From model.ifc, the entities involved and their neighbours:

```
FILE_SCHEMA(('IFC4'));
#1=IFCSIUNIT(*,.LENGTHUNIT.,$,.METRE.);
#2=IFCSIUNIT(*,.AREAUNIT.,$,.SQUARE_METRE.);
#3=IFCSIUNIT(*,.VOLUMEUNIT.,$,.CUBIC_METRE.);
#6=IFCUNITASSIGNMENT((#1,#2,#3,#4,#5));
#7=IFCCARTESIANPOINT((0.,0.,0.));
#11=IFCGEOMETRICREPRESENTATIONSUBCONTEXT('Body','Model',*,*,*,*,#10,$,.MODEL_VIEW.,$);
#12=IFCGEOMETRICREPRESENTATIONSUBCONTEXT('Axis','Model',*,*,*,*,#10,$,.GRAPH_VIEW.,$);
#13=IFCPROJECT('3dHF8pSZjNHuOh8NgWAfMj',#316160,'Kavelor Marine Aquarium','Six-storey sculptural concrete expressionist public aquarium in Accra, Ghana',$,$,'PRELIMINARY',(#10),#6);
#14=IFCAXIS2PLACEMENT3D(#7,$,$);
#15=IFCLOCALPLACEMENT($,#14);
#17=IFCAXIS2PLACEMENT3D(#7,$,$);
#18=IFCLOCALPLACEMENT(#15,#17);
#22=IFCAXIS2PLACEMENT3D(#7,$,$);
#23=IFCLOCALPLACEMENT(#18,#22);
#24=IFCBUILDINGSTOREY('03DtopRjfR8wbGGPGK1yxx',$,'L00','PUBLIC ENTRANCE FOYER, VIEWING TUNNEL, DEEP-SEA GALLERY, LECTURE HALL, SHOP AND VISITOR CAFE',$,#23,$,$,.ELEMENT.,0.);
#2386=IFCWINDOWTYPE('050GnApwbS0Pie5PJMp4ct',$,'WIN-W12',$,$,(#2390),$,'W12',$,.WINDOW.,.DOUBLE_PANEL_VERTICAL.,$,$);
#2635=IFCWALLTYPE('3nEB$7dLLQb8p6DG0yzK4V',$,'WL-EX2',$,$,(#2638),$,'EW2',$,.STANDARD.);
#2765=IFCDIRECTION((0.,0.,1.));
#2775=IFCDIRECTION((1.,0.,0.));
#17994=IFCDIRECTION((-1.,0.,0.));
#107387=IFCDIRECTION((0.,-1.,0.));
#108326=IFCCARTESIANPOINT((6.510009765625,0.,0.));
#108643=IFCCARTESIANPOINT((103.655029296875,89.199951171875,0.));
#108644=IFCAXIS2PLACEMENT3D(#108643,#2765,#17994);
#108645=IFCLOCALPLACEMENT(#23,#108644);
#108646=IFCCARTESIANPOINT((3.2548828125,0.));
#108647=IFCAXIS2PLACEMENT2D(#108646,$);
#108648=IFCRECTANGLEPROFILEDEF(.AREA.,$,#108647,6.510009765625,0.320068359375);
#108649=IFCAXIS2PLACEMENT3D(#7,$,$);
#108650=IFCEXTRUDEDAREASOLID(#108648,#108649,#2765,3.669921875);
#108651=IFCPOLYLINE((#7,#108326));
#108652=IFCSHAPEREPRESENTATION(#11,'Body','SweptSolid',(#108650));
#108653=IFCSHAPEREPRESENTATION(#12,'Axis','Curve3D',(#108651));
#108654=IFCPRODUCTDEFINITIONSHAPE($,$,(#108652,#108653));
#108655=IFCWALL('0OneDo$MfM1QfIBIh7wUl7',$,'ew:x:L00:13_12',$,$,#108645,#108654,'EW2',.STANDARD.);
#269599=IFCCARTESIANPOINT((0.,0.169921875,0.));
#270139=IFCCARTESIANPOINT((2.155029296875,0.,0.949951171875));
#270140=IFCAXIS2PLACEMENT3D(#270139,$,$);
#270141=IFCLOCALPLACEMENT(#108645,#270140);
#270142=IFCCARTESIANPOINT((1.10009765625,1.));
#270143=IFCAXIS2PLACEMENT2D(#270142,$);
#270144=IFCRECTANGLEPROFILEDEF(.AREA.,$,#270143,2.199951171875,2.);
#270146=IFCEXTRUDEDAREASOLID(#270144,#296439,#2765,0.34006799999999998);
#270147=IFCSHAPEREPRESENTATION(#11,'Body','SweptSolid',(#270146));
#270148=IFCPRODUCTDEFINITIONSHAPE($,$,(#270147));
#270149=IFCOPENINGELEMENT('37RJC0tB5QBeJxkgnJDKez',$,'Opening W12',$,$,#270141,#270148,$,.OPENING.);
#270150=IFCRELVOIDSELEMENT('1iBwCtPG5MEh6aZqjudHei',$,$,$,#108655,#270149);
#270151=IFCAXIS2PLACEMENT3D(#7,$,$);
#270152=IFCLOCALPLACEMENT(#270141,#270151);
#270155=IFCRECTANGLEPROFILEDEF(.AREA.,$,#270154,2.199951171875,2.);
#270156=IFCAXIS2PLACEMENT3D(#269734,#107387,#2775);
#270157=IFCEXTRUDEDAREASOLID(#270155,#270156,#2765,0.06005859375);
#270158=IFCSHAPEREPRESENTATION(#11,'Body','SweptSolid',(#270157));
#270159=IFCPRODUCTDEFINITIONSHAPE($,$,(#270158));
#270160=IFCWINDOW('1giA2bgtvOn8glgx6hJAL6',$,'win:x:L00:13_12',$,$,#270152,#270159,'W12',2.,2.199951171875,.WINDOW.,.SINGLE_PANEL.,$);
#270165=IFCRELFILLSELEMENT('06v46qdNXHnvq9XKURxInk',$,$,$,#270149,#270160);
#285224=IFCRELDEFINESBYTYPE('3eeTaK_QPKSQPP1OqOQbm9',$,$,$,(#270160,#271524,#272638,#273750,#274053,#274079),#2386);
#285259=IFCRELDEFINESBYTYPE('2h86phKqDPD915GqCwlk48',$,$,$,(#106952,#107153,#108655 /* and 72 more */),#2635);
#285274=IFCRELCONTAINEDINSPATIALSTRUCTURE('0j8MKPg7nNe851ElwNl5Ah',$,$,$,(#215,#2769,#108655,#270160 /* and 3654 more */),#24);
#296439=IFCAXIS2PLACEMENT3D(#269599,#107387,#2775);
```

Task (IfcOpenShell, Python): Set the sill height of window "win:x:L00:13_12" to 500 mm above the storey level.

```python
import numpy as np
import ifcopenshell
import ifcopenshell.api.geometry
import ifcopenshell.geom
import ifcopenshell.util.element
import ifcopenshell.util.placement
import ifcopenshell.util.shape
import ifcopenshell.util.unit

model = ifcopenshell.open("model.ifc")
unit_scale = ifcopenshell.util.unit.calculate_unit_scale(model)

window = model.by_guid("1giA2bgtvOn8glgx6hJAL6")
opening = window.FillsVoids[0].RelatingOpeningElement
storey = ifcopenshell.util.element.get_container(window, ifc_class="IfcBuildingStorey")
level = ifcopenshell.util.placement.get_local_placement(storey.ObjectPlacement)[2, 3]

# The opening's origin need not be at the sill, so measure its lowest point.
shape = ifcopenshell.geom.create_shape(ifcopenshell.geom.settings(), opening)
bottom = ifcopenshell.util.shape.get_shape_bottom_elevation(shape, shape.geometry) / unit_scale
dz = level + 0.5 / unit_scale - bottom

shift = np.array([0.0, 0.0, dz])
# The window is placed relative to its opening, so it follows when the opening moves.
matrix = ifcopenshell.util.placement.get_local_placement(opening.ObjectPlacement)
matrix[:3, 3] += shift
ifcopenshell.api.geometry.edit_object_placement(
    model, product=opening, matrix=matrix, is_si=False, should_transform_children=True
)

print(f"moved by {dz * unit_scale:+.3f} m")

model.write("model_rev.ifc")
```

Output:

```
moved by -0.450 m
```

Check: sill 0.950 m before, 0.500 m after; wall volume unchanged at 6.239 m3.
